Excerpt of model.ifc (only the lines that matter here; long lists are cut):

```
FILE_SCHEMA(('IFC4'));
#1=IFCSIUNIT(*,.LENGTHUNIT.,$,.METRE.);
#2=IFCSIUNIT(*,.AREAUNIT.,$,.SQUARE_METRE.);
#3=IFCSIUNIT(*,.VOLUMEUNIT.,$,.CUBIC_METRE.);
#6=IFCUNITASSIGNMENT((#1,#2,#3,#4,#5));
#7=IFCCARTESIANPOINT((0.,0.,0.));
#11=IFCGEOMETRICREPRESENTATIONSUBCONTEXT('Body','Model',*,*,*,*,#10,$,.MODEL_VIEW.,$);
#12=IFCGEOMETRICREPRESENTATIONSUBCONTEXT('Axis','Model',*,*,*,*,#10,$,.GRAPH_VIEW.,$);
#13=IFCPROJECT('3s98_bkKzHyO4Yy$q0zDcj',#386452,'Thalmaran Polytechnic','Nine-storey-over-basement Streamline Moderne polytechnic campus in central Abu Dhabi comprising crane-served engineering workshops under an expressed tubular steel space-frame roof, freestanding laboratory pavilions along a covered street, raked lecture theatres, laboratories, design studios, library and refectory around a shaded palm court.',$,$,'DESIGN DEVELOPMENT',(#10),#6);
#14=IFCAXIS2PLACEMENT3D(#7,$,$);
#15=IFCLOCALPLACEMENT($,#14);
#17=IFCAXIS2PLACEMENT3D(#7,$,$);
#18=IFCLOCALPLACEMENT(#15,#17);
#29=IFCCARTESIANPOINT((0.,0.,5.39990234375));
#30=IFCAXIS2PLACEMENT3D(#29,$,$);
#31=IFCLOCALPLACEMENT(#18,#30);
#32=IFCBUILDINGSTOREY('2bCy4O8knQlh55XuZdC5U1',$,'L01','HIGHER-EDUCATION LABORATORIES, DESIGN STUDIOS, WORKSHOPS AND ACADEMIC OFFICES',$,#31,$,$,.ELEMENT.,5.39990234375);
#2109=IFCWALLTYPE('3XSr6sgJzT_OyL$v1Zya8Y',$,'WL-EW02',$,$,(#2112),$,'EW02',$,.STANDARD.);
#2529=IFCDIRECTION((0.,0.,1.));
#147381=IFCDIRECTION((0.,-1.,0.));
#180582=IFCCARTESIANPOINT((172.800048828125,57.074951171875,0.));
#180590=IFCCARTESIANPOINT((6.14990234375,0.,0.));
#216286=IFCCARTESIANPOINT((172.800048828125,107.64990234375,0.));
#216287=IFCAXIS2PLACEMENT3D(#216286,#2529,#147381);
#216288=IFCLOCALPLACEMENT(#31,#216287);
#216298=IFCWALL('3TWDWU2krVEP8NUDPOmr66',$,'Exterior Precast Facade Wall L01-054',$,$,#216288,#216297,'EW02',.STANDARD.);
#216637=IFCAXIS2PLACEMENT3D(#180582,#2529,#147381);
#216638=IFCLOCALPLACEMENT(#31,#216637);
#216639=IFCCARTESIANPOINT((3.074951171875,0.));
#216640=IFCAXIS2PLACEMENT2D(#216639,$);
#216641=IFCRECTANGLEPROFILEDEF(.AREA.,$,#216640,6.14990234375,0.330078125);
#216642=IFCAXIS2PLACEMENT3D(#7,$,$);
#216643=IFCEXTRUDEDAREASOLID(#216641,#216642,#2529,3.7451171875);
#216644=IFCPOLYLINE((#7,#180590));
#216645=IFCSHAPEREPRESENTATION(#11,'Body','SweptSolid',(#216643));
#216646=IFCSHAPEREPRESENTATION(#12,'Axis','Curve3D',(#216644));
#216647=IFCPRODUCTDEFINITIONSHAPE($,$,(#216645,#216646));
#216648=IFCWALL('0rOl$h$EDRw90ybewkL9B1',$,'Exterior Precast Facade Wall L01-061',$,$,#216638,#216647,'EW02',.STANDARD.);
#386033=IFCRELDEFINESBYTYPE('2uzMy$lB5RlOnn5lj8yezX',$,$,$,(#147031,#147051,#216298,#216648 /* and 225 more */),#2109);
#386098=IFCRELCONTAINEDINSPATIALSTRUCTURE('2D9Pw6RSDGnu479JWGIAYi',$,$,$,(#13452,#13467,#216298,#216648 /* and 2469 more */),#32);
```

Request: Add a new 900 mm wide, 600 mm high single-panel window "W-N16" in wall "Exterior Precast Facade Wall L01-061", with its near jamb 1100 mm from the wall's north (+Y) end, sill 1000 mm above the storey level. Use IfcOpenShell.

```python
import numpy as np
import ifcopenshell
import ifcopenshell.api.feature
import ifcopenshell.api.geometry
import ifcopenshell.api.root
import ifcopenshell.api.spatial
import ifcopenshell.geom
import ifcopenshell.util.element
import ifcopenshell.util.placement
import ifcopenshell.util.representation
import ifcopenshell.util.shape
import ifcopenshell.util.unit

model = ifcopenshell.open("model.ifc")
unit_scale = ifcopenshell.util.unit.calculate_unit_scale(model)
settings = ifcopenshell.geom.settings()


def volume(element):
    """Net volume in cubic metres, openings subtracted."""
    shape = ifcopenshell.geom.create_shape(settings, element)
    return ifcopenshell.util.shape.get_volume(shape.geometry)


wall = model.by_guid("0rOl$h$EDRw90ybewkL9B1")
storey = ifcopenshell.util.element.get_container(wall, ifc_class="IfcBuildingStorey")
context = ifcopenshell.util.representation.get_context(model, "Model", "Body", "MODEL_VIEW")
before = volume(wall)

width, height, from_end, sill = 0.9, 0.6, 1.1, 1  # metres

# The wall runs along its own X axis, and the end named is its -X end.
wall_shape = ifcopenshell.geom.create_shape(settings, wall)
x, y, z = ifcopenshell.util.shape.get_vertices(wall_shape.geometry).T
start = x.min() + from_end
face, thickness = float(y.min()), float(y.max() - y.min())
wall_matrix = ifcopenshell.util.placement.get_local_placement(wall.ObjectPlacement)
level = ifcopenshell.util.placement.get_local_placement(storey.ObjectPlacement)[2, 3]


def in_wall(x, y):
    """Placement at x, y metres in the wall's axes, at sill height."""
    matrix = wall_matrix.copy()
    matrix[:, 3] = wall_matrix @ np.array([x / unit_scale, y / unit_scale, 0.0, 1.0])
    matrix[2, 3] = level + sill / unit_scale
    return matrix


# Opening: a box that overshoots both wall faces by 50 mm.
opening = ifcopenshell.api.root.create_entity(model, ifc_class="IfcOpeningElement", predefined_type="OPENING")
box = ifcopenshell.api.geometry.add_wall_representation(
    model, context=context, length=width, height=height, thickness=thickness + 0.1
)
ifcopenshell.api.geometry.assign_representation(model, product=opening, representation=box)
ifcopenshell.api.geometry.edit_object_placement(model, product=opening, matrix=in_wall(start, face - 0.05), is_si=False)
ifcopenshell.api.feature.add_feature(model, feature=opening, element=wall)

window = ifcopenshell.api.root.create_entity(model, ifc_class="IfcWindow", name="W-N16", predefined_type="WINDOW")
window.OverallWidth, window.OverallHeight = width / unit_scale, height / unit_scale
window.PartitioningType = "SINGLE_PANEL"
body = ifcopenshell.api.geometry.add_window_representation(
    model,
    context=context,
    overall_width=window.OverallWidth,
    overall_height=window.OverallHeight,
    partition_type="SINGLE_PANEL",
)
ifcopenshell.api.geometry.assign_representation(model, product=window, representation=body)
ifcopenshell.api.spatial.assign_container(model, products=[window], relating_structure=storey)
ifcopenshell.api.feature.add_filling(model, opening=opening, element=window)

# Centre the window in the wall's thickness.
ifcopenshell.api.geometry.edit_object_placement(model, product=window, matrix=in_wall(start, face), is_si=False)
window_shape = ifcopenshell.geom.create_shape(settings, window)
depth = ifcopenshell.util.shape.get_vertices(window_shape.geometry)[:, 1]
offset = face + thickness / 2 - (depth.min() + depth.max()) / 2
ifcopenshell.api.geometry.edit_object_placement(model, product=window, matrix=in_wall(start, offset), is_si=False)

after = volume(wall)

print(f"wall volume {before:.3f} -> {after:.3f} m3")

model.write("model_v2.ifc")
```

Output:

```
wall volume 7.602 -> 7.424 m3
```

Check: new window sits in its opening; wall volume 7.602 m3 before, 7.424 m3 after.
